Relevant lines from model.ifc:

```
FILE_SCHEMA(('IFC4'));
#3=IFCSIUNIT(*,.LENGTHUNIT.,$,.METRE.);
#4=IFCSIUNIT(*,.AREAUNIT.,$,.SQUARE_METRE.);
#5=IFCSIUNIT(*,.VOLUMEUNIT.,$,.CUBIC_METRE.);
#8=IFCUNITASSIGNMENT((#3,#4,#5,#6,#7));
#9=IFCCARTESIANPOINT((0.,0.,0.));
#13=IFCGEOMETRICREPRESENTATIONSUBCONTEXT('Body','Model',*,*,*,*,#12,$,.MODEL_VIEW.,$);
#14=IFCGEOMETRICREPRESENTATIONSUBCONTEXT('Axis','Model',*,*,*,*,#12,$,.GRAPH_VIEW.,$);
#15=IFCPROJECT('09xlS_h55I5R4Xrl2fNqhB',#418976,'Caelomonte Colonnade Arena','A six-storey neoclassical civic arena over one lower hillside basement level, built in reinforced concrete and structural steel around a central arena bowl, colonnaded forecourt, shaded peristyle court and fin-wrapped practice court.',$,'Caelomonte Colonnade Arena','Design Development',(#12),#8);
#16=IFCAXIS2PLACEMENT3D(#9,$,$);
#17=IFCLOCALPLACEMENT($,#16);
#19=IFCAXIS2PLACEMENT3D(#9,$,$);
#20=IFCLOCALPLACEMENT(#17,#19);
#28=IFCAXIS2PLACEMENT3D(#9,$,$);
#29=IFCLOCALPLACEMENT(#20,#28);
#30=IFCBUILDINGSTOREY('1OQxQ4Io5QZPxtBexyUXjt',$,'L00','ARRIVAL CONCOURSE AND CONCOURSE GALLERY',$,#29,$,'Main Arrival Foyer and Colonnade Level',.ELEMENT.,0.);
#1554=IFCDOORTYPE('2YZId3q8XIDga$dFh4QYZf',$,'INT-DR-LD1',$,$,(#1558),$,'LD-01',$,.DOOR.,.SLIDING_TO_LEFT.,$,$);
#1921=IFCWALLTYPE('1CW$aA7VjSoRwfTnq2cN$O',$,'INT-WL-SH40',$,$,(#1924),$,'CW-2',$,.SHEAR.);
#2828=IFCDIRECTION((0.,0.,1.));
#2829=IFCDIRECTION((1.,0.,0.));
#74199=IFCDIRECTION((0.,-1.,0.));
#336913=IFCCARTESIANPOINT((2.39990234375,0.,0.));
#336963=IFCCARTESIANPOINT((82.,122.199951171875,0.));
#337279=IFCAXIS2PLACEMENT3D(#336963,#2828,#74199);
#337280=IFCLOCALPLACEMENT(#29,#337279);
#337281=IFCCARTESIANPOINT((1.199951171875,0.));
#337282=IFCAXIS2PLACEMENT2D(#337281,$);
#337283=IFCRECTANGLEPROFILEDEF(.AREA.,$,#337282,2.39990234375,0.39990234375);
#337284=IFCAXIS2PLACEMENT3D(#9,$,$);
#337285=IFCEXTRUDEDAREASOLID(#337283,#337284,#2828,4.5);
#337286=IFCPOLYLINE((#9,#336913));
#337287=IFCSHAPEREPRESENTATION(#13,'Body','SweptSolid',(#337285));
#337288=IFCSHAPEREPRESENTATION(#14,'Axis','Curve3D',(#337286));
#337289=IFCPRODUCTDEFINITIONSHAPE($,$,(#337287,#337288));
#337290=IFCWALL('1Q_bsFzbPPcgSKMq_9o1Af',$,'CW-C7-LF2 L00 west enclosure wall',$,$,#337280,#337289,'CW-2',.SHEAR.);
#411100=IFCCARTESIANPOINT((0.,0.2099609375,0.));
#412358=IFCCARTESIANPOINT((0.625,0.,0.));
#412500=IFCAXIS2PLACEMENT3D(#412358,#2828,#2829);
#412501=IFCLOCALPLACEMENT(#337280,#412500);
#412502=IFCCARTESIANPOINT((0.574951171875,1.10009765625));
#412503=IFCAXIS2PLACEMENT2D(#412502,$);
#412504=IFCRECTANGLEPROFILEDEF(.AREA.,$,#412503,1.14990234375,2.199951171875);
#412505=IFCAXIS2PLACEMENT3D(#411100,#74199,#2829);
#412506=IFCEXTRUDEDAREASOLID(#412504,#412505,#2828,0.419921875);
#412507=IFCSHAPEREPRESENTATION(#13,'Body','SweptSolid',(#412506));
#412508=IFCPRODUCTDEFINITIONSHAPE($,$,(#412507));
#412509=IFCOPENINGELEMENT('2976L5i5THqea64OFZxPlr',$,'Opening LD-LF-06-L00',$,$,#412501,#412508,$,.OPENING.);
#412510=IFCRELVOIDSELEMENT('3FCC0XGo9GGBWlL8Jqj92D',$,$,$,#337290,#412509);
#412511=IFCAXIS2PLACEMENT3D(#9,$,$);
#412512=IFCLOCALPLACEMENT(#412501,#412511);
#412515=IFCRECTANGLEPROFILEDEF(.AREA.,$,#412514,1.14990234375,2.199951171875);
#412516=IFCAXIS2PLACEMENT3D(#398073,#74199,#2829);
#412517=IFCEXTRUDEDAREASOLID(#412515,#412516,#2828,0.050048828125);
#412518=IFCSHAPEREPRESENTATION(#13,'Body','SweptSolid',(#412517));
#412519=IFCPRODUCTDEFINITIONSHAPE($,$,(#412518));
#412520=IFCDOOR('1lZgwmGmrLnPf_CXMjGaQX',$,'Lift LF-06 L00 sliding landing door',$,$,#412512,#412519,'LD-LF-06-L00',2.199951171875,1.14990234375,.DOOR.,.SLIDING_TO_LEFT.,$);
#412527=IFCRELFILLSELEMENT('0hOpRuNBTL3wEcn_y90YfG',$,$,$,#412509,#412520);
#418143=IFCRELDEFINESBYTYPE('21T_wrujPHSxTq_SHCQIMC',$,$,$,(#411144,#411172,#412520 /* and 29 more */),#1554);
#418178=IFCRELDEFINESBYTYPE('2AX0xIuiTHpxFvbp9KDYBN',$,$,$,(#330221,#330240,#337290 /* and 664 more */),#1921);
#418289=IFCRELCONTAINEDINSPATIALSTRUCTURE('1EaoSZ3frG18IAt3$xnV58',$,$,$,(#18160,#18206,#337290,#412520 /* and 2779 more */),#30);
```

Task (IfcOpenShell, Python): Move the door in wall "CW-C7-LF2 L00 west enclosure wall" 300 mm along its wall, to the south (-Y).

```python
import ifcopenshell
import ifcopenshell.api.geometry
import ifcopenshell.util.placement
import ifcopenshell.util.unit

model = ifcopenshell.open("model.ifc")
unit_scale = ifcopenshell.util.unit.calculate_unit_scale(model)

door = model.by_guid("1lZgwmGmrLnPf_CXMjGaQX")
opening = door.FillsVoids[0].RelatingOpeningElement
wall = opening.VoidsElements[0].RelatingBuildingElement

wall_matrix = ifcopenshell.util.placement.get_local_placement(wall.ObjectPlacement)
shift = wall_matrix[:3, 0] * 0.3 / unit_scale
before = ifcopenshell.util.placement.get_local_placement(door.ObjectPlacement)[:3, 3].copy()

# The door is placed relative to its opening, so it follows when the opening moves.
matrix = ifcopenshell.util.placement.get_local_placement(opening.ObjectPlacement)
matrix[:3, 3] += shift
ifcopenshell.api.geometry.edit_object_placement(
    model, product=opening, matrix=matrix, is_si=False, should_transform_children=True
)

after = ifcopenshell.util.placement.get_local_placement(door.ObjectPlacement)[:3, 3]
print("door moved by", (after - before).round(3) + 0.0)

model.write("model_rev.ifc")
```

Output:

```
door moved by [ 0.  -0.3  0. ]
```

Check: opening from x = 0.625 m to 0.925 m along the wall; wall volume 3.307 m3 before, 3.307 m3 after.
